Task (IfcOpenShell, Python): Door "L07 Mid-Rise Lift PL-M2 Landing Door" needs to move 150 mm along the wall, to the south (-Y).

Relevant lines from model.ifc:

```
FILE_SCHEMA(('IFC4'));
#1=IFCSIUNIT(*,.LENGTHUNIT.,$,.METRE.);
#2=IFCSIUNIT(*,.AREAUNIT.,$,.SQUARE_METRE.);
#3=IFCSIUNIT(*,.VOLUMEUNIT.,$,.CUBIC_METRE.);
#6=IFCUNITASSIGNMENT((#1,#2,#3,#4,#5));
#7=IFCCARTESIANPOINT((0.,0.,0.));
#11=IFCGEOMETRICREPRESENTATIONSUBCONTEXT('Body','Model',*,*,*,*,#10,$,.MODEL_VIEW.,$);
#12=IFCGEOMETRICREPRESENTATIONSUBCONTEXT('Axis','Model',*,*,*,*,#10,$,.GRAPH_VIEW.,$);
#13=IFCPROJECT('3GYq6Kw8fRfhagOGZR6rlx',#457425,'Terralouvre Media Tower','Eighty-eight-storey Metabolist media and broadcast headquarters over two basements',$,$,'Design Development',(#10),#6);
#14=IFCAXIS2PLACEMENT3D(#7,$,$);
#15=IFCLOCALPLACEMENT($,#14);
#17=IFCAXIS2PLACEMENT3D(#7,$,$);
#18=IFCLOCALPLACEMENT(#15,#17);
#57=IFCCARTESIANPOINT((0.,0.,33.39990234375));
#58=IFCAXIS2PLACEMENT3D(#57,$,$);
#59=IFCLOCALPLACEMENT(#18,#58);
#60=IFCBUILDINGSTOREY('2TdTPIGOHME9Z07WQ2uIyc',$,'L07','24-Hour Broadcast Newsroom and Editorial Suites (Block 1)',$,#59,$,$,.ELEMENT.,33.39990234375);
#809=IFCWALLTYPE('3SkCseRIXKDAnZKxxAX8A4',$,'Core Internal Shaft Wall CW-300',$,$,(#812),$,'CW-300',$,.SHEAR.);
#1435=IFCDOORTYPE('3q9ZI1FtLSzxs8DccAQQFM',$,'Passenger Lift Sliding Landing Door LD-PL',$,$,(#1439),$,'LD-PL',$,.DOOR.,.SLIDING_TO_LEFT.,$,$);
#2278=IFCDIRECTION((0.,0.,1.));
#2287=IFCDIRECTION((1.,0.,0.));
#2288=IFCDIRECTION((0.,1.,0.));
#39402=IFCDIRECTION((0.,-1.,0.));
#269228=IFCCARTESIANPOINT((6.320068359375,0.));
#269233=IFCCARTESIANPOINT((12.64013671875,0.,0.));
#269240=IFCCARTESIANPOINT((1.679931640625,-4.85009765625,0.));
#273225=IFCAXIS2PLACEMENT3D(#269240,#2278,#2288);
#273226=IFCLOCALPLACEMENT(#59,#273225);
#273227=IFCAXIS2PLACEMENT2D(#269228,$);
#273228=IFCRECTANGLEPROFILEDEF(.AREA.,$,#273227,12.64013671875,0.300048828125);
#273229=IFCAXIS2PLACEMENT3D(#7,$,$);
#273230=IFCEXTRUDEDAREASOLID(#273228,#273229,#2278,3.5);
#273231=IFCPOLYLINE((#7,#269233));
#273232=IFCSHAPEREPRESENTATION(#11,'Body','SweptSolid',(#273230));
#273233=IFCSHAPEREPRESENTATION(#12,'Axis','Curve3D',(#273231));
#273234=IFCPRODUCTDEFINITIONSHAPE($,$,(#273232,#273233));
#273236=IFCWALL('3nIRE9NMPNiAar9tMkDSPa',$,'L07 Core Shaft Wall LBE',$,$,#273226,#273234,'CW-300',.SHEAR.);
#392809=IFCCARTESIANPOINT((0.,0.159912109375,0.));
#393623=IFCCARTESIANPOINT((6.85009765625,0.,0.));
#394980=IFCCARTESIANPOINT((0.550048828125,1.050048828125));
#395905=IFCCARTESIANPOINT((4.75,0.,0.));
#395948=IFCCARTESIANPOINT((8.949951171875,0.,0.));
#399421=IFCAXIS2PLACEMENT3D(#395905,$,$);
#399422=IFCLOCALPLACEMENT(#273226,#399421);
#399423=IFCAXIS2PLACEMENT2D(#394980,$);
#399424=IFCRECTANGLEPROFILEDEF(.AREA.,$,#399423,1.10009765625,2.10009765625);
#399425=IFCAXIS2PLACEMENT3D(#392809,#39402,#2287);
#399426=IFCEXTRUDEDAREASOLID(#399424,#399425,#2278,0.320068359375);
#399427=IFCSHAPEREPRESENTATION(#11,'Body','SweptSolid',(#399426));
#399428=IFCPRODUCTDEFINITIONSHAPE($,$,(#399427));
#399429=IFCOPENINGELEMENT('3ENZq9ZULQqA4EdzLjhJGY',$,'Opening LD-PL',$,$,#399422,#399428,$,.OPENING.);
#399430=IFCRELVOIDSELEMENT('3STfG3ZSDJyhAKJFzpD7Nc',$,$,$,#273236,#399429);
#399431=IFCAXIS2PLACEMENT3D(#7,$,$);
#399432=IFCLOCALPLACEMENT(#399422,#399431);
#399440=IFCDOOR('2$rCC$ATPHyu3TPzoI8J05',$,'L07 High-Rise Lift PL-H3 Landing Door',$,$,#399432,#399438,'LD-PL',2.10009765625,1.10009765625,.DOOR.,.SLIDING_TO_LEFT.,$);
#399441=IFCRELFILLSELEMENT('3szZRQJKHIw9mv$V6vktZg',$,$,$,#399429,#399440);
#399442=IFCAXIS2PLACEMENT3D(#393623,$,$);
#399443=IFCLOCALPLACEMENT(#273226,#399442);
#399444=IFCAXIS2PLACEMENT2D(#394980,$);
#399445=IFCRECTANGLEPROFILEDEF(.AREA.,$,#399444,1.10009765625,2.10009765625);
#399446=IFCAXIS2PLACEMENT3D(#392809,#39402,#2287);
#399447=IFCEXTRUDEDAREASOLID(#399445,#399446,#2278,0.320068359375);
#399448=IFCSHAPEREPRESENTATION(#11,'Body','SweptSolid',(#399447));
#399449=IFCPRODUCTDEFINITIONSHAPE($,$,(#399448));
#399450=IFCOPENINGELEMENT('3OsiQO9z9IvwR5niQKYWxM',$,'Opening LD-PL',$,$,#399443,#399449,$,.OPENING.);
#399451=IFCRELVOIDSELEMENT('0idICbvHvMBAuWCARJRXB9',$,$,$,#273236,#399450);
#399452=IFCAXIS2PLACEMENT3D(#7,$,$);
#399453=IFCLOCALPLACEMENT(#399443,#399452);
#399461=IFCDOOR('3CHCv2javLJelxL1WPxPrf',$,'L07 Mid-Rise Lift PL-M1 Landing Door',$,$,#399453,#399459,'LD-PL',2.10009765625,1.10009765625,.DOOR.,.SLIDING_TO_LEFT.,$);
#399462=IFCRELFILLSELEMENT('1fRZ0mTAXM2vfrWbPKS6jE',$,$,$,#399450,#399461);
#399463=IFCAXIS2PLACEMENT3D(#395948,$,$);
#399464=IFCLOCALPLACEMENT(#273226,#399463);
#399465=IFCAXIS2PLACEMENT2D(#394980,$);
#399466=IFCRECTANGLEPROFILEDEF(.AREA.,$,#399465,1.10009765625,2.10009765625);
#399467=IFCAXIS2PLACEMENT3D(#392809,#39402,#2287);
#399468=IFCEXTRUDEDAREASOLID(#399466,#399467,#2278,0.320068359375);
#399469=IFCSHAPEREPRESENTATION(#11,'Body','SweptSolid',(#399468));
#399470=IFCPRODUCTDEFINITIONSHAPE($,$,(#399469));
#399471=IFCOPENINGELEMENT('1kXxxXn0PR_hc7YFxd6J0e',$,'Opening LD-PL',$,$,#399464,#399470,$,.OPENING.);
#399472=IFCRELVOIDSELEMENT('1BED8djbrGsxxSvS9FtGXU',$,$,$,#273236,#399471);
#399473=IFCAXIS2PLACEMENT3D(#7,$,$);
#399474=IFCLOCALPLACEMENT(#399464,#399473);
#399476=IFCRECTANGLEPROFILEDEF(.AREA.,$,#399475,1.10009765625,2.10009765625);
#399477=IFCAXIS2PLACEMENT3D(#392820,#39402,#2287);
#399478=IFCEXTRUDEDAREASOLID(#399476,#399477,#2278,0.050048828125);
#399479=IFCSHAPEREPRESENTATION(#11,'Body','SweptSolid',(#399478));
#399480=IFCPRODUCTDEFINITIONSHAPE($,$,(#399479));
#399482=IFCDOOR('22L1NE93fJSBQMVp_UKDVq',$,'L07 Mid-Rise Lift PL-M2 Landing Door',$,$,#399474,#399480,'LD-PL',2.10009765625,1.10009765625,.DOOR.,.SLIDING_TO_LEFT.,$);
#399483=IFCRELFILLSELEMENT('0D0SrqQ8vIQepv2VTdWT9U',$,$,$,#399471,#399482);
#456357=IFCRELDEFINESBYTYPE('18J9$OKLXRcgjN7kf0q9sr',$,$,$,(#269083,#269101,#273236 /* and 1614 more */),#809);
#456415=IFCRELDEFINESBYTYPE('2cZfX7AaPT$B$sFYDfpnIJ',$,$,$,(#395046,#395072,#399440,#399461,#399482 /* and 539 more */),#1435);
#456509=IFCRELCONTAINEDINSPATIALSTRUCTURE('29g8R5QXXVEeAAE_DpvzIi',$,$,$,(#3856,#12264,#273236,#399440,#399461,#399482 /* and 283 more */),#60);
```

```python
import ifcopenshell
import ifcopenshell.api.geometry
import ifcopenshell.util.placement

model = ifcopenshell.open("model.ifc")

door = model.by_guid("22L1NE93fJSBQMVp_UKDVq")
opening = door.FillsVoids[0].RelatingOpeningElement
wall = opening.VoidsElements[0].RelatingBuildingElement

wall_matrix = ifcopenshell.util.placement.get_local_placement(wall.ObjectPlacement)
shift = wall_matrix[:3, 0] * -0.15
before = ifcopenshell.util.placement.get_local_placement(door.ObjectPlacement)[:3, 3].copy()

# The door is placed relative to its opening, so it follows when the opening moves.
matrix = ifcopenshell.util.placement.get_local_placement(opening.ObjectPlacement)
matrix[:3, 3] += shift
ifcopenshell.api.geometry.edit_object_placement(
    model, product=opening, matrix=matrix, is_si=False, should_transform_children=True
)

after = ifcopenshell.util.placement.get_local_placement(door.ObjectPlacement)[:3, 3]
print("door moved by", (after - before).round(3) + 0.0)

model.write("model-out.ifc")
```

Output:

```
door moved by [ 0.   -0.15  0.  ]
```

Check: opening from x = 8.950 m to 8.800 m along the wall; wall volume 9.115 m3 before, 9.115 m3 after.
